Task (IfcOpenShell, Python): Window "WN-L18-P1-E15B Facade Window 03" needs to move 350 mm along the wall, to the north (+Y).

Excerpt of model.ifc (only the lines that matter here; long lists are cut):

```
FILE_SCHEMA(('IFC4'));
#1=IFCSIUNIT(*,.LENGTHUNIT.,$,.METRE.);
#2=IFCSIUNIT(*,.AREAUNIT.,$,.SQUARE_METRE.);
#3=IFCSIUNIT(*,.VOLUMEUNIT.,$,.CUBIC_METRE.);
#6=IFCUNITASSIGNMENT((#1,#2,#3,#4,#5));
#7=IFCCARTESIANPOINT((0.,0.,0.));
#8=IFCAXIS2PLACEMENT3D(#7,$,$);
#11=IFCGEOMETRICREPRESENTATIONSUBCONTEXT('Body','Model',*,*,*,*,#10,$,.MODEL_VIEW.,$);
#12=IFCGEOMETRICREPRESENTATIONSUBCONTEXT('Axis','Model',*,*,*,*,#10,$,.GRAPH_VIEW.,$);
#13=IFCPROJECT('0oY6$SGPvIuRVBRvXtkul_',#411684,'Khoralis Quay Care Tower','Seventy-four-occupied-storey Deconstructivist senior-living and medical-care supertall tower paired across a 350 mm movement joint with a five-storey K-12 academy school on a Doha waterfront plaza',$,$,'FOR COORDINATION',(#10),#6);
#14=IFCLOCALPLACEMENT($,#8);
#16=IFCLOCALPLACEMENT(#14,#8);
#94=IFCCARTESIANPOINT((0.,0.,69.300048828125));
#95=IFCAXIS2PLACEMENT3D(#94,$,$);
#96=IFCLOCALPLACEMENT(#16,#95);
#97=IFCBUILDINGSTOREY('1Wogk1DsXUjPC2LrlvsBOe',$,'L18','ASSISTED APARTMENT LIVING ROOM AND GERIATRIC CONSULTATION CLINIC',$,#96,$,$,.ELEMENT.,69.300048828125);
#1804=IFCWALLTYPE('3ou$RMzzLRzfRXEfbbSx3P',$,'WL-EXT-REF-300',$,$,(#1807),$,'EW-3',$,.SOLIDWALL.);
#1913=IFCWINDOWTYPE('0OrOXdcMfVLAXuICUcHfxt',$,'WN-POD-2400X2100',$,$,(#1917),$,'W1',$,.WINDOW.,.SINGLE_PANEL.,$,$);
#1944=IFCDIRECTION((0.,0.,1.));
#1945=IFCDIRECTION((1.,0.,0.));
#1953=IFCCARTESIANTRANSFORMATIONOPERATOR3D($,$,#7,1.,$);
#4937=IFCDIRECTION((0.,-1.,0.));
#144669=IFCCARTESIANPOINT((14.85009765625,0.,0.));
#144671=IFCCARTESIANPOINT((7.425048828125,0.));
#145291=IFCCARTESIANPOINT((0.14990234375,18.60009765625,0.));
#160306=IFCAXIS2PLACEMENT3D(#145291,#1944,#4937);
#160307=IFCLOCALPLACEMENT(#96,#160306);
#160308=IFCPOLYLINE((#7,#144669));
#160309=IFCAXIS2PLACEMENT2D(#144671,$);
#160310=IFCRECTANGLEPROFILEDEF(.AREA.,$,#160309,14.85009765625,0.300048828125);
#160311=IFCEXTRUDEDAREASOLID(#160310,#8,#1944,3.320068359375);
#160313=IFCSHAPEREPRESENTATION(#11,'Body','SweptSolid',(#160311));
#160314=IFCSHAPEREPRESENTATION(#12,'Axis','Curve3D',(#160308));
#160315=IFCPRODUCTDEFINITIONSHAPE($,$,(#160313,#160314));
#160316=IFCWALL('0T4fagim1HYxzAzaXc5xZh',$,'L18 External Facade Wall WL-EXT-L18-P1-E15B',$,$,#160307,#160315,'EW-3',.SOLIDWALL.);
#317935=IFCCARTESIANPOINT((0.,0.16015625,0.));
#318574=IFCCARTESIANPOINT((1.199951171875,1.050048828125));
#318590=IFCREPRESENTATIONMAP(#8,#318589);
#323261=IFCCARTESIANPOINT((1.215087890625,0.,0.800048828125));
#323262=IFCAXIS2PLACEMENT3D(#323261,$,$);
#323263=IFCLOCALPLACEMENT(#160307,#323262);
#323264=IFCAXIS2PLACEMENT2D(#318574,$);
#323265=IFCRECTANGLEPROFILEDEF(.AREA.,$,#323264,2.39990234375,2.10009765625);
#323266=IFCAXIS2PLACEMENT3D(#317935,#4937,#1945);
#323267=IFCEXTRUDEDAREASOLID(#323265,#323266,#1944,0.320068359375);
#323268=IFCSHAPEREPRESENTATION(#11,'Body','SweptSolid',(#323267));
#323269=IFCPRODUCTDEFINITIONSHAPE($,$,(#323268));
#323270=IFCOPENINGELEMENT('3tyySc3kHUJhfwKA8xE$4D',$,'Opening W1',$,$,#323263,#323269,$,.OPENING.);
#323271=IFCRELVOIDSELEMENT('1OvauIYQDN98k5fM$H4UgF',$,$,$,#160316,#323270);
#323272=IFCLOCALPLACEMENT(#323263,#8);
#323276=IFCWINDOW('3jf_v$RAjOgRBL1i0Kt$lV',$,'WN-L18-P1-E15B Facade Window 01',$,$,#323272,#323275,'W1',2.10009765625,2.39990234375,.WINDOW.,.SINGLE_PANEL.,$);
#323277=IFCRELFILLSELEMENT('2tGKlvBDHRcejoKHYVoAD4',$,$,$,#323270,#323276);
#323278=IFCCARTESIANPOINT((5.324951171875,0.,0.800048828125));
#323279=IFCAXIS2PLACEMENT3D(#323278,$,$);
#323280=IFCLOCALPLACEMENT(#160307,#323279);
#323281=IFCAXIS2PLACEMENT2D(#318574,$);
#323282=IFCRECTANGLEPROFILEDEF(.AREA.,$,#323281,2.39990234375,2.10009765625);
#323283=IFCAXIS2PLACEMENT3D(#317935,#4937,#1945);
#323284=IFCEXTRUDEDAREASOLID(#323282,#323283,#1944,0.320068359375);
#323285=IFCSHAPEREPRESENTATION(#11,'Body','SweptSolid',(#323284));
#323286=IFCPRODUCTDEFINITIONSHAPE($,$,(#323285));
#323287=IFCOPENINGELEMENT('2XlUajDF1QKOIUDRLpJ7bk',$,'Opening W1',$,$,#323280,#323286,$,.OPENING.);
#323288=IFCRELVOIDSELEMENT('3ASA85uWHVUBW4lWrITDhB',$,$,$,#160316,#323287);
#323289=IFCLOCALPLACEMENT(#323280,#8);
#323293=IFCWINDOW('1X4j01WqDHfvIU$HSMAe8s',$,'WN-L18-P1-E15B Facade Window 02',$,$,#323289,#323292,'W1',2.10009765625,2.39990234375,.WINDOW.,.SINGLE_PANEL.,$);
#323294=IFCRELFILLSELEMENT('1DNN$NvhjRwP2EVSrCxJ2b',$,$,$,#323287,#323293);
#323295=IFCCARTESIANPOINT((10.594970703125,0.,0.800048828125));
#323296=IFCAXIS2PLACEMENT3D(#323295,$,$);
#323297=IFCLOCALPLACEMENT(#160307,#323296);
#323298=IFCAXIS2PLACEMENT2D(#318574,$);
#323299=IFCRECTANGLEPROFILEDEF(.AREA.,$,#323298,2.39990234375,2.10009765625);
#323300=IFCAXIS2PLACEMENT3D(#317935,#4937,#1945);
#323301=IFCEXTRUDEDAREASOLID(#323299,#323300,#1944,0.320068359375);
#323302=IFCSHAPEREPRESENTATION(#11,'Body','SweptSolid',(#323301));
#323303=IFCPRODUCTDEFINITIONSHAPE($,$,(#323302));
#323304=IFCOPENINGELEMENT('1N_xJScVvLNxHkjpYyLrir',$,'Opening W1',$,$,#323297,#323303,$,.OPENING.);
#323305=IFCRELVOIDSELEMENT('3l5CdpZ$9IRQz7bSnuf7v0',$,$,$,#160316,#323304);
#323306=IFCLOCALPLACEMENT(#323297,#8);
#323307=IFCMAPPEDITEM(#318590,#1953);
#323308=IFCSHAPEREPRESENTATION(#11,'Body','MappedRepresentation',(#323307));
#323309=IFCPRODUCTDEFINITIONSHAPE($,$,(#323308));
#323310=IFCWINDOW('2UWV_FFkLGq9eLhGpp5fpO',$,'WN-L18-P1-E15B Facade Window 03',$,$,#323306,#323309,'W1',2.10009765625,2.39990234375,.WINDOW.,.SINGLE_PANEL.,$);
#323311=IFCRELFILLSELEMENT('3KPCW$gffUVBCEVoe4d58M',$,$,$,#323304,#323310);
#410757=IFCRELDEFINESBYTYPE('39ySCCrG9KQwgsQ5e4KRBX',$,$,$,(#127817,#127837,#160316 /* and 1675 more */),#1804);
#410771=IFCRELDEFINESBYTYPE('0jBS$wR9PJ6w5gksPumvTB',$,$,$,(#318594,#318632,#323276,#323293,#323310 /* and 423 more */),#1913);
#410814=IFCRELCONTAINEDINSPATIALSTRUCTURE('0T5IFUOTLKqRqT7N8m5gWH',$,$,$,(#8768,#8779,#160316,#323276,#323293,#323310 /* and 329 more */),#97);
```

```python
import ifcopenshell
import ifcopenshell.api.geometry
import ifcopenshell.util.placement
import ifcopenshell.util.unit

model = ifcopenshell.open("model.ifc")
unit_scale = ifcopenshell.util.unit.calculate_unit_scale(model)

window = model.by_id(323310)
opening = window.FillsVoids[0].RelatingOpeningElement
wall = opening.VoidsElements[0].RelatingBuildingElement

wall_matrix = ifcopenshell.util.placement.get_local_placement(wall.ObjectPlacement)
shift = wall_matrix[:3, 0] * -0.35 / unit_scale
before = ifcopenshell.util.placement.get_local_placement(window.ObjectPlacement)[:3, 3].copy()

# The window is placed relative to its opening, so it follows when the opening moves.
matrix = ifcopenshell.util.placement.get_local_placement(opening.ObjectPlacement)
matrix[:3, 3] += shift
ifcopenshell.api.geometry.edit_object_placement(
    model, product=opening, matrix=matrix, is_si=False, should_transform_children=True
)

after = ifcopenshell.util.placement.get_local_placement(window.ObjectPlacement)[:3, 3]
print("window moved by", (after - before).round(3) + 0.0)

model.write("model_updated.ifc")
```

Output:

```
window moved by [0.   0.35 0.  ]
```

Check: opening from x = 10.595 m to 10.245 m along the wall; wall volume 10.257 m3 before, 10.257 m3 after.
